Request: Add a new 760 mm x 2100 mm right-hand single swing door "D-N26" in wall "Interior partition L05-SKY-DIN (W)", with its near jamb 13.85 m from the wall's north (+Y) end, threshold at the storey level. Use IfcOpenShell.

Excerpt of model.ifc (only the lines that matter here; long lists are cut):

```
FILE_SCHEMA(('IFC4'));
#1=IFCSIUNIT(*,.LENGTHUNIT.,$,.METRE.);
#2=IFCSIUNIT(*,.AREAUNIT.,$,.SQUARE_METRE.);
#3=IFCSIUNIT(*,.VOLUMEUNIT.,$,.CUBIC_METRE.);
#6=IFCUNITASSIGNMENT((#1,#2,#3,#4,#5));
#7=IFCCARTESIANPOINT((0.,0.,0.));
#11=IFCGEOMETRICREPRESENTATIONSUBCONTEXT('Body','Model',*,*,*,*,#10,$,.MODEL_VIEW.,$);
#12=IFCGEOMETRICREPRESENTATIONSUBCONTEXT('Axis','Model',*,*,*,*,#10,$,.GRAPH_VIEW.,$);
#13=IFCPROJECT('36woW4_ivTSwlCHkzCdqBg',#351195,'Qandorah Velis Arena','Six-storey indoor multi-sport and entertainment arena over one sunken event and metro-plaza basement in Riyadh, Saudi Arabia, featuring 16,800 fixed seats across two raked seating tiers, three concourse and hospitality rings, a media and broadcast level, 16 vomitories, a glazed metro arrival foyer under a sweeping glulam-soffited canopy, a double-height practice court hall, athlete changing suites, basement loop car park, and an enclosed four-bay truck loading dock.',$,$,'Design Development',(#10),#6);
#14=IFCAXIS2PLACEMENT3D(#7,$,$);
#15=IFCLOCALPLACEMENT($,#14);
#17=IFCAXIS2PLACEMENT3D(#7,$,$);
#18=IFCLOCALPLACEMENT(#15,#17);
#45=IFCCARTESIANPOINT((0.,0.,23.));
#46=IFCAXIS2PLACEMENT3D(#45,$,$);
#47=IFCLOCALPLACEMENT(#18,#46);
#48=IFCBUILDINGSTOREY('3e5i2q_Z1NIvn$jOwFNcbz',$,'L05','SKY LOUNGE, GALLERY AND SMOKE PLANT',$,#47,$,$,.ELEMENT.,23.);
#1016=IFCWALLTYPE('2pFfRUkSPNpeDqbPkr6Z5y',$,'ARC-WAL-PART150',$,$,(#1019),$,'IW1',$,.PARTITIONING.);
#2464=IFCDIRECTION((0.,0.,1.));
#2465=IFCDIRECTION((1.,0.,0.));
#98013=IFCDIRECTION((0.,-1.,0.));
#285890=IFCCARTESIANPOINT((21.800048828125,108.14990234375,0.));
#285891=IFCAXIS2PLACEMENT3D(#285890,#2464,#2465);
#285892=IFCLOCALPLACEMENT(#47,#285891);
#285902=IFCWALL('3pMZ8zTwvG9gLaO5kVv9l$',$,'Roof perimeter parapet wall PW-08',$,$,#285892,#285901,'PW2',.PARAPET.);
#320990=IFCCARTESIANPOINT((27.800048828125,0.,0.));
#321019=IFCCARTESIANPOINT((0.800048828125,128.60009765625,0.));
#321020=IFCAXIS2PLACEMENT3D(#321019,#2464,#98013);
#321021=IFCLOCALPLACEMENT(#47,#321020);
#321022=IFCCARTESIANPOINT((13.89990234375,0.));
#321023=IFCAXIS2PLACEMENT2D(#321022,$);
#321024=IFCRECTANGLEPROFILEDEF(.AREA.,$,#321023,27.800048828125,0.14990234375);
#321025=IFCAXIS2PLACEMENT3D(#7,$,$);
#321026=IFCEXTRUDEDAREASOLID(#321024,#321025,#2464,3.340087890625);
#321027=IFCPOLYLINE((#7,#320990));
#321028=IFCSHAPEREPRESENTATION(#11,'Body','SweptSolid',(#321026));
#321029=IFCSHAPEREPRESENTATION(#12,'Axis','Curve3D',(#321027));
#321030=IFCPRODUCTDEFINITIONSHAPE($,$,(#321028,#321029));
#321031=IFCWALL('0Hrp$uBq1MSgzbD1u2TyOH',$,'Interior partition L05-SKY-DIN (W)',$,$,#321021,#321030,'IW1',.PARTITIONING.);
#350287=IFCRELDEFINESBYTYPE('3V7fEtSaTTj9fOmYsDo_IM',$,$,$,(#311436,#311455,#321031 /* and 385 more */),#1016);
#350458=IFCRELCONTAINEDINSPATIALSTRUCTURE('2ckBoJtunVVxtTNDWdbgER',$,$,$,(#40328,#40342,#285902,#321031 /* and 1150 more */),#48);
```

```python
import numpy as np
import ifcopenshell
import ifcopenshell.api.feature
import ifcopenshell.api.geometry
import ifcopenshell.api.root
import ifcopenshell.api.spatial
import ifcopenshell.geom
import ifcopenshell.util.element
import ifcopenshell.util.placement
import ifcopenshell.util.representation
import ifcopenshell.util.shape
import ifcopenshell.util.unit

model = ifcopenshell.open("model.ifc")
unit_scale = ifcopenshell.util.unit.calculate_unit_scale(model)
settings = ifcopenshell.geom.settings()


def volume(element):
    """Net volume in cubic metres, openings subtracted."""
    shape = ifcopenshell.geom.create_shape(settings, element)
    return ifcopenshell.util.shape.get_volume(shape.geometry)


wall = model.by_id(321031)
storey = ifcopenshell.util.element.get_container(wall, ifc_class="IfcBuildingStorey")
context = ifcopenshell.util.representation.get_context(model, "Model", "Body", "MODEL_VIEW")
before = volume(wall)

width, height, from_end, sill = 0.76, 2.1, 13.85, 0.0  # metres

# The wall runs along its own X axis, and the end named is its -X end.
wall_shape = ifcopenshell.geom.create_shape(settings, wall)
x, y, z = ifcopenshell.util.shape.get_vertices(wall_shape.geometry).T
start = x.min() + from_end
face, thickness = float(y.min()), float(y.max() - y.min())
wall_matrix = ifcopenshell.util.placement.get_local_placement(wall.ObjectPlacement)
level = ifcopenshell.util.placement.get_local_placement(storey.ObjectPlacement)[2, 3]


def in_wall(x, y):
    """Placement at x, y metres in the wall's axes, at sill height."""
    matrix = wall_matrix.copy()
    matrix[:, 3] = wall_matrix @ np.array([x / unit_scale, y / unit_scale, 0.0, 1.0])
    matrix[2, 3] = level + sill / unit_scale
    return matrix


# Opening: a box that overshoots both wall faces by 50 mm.
opening = ifcopenshell.api.root.create_entity(model, ifc_class="IfcOpeningElement", predefined_type="OPENING")
box = ifcopenshell.api.geometry.add_wall_representation(
    model, context=context, length=width, height=height, thickness=thickness + 0.1
)
ifcopenshell.api.geometry.assign_representation(model, product=opening, representation=box)
ifcopenshell.api.geometry.edit_object_placement(model, product=opening, matrix=in_wall(start, face - 0.05), is_si=False)
ifcopenshell.api.feature.add_feature(model, feature=opening, element=wall)

door = ifcopenshell.api.root.create_entity(model, ifc_class="IfcDoor", name="D-N26", predefined_type="DOOR")
door.OverallWidth, door.OverallHeight = width / unit_scale, height / unit_scale
door.OperationType = "SINGLE_SWING_RIGHT"
body = ifcopenshell.api.geometry.add_door_representation(
    model,
    context=context,
    overall_width=door.OverallWidth,
    overall_height=door.OverallHeight,
    operation_type="SINGLE_SWING_RIGHT",
    lining_properties={"LiningDepth": thickness / unit_scale, "ThresholdDepth": thickness / unit_scale},
)
ifcopenshell.api.geometry.assign_representation(model, product=door, representation=body)
ifcopenshell.api.spatial.assign_container(model, products=[door], relating_structure=storey)
ifcopenshell.api.feature.add_filling(model, opening=opening, element=door)

# The lining spans the wall, so the door starts at the wall face.
ifcopenshell.api.geometry.edit_object_placement(model, product=door, matrix=in_wall(start, face), is_si=False)

after = volume(wall)

print(f"wall volume {before:.3f} -> {after:.3f} m3")

model.write("model_edited.ifc")
```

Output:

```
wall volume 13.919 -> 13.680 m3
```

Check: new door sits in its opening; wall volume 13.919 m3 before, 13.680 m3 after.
